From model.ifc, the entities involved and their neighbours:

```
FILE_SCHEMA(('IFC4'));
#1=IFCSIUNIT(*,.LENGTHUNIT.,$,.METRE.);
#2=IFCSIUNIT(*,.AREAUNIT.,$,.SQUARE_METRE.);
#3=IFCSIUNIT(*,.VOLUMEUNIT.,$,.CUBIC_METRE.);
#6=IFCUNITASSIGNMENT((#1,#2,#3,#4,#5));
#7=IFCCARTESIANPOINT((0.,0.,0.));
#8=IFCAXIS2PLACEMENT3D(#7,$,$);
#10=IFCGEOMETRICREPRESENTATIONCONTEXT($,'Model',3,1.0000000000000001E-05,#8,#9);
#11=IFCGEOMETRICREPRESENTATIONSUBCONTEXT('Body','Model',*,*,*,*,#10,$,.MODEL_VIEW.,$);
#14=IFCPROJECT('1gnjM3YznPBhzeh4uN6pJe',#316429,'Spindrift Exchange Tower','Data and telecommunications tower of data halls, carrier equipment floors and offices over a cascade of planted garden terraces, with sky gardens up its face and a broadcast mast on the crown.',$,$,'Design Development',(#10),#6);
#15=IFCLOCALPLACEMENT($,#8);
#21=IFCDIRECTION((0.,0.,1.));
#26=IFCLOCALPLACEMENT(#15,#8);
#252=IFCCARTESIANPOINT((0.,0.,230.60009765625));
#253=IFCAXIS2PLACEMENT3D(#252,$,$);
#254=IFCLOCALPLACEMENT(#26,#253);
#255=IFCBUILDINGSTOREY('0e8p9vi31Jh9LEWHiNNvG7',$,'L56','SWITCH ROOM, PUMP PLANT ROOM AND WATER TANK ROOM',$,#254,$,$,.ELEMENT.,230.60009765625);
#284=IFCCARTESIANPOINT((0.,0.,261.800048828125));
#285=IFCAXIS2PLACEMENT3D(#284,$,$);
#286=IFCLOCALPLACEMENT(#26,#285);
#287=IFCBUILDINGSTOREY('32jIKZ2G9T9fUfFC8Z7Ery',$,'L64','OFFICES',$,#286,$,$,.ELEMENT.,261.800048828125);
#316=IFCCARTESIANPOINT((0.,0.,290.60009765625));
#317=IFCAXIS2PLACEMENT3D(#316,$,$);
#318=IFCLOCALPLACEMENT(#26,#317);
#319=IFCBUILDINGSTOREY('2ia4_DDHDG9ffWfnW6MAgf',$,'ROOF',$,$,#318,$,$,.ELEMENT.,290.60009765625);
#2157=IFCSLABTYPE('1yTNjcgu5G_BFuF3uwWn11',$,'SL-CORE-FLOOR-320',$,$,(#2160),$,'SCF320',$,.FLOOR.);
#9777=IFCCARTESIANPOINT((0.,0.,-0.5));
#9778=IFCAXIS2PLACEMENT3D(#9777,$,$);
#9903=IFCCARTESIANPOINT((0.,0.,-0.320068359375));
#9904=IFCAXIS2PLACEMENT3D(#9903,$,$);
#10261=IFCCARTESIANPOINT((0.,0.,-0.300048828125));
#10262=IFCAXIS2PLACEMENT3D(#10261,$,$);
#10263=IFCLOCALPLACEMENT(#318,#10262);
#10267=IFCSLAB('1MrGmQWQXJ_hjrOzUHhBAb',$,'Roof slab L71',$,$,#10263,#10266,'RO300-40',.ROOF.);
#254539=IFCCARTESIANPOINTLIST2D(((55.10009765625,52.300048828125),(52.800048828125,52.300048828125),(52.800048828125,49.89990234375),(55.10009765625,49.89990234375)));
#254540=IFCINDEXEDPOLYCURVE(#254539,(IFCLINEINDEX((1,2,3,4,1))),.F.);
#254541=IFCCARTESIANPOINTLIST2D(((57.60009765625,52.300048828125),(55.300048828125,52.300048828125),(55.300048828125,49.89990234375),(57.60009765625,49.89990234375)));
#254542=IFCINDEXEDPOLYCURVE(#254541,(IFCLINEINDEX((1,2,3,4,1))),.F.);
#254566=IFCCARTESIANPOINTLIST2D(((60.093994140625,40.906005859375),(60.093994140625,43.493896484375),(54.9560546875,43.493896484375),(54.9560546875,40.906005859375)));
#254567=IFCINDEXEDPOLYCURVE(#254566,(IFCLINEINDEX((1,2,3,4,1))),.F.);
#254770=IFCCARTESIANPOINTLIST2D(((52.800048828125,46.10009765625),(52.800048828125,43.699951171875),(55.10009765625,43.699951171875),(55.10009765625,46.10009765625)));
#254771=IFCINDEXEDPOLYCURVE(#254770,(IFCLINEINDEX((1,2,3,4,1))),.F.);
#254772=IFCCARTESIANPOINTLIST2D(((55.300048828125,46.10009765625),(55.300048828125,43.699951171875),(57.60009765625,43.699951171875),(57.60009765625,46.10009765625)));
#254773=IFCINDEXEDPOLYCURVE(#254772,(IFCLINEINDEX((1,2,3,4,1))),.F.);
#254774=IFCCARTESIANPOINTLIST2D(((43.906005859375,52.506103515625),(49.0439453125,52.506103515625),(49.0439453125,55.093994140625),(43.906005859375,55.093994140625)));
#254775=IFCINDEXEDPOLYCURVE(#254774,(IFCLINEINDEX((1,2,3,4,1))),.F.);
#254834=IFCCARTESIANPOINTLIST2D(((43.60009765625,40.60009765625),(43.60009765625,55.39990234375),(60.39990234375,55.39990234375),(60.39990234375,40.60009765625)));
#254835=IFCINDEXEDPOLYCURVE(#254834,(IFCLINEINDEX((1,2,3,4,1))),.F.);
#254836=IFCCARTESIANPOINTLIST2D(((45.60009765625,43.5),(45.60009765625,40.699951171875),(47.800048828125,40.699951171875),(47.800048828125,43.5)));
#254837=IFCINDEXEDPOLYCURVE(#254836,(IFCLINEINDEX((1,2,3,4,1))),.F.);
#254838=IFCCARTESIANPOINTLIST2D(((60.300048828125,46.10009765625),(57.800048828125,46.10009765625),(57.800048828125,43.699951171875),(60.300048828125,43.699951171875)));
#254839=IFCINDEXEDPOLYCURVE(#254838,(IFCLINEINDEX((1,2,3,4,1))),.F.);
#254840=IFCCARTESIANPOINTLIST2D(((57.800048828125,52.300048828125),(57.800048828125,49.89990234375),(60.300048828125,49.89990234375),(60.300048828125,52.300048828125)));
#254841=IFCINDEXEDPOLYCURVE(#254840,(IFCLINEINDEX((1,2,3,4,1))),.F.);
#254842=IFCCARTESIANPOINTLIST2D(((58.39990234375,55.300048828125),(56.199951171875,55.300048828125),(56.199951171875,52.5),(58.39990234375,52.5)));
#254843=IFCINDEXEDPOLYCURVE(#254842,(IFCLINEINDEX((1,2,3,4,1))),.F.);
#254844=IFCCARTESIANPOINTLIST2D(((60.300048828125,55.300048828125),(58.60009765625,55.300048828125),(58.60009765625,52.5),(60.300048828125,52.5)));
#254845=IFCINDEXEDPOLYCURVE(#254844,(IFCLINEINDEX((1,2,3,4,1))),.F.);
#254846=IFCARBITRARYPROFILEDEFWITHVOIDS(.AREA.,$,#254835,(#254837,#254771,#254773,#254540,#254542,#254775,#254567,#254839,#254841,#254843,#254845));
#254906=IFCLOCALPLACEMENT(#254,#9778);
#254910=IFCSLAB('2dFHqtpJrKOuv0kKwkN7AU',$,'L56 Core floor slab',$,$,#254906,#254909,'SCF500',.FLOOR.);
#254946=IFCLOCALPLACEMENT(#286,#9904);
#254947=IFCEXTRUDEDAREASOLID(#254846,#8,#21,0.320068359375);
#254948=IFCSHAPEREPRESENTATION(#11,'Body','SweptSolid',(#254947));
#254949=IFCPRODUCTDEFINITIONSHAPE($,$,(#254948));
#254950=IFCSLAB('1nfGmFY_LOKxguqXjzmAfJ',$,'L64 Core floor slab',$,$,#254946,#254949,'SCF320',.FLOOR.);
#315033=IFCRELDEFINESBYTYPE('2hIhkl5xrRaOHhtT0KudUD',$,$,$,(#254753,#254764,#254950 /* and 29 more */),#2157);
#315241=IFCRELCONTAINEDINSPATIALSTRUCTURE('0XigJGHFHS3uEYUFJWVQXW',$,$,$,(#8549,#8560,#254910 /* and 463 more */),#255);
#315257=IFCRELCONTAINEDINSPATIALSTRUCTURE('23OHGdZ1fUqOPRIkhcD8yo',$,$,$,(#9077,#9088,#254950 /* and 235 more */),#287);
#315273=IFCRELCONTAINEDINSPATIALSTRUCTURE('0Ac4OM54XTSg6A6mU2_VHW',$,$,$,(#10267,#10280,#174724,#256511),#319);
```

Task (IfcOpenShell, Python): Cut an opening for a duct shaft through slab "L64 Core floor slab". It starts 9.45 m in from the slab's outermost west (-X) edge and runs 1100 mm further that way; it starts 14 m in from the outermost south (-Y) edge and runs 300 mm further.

```python
import numpy as np
import ifcopenshell
import ifcopenshell.api.feature
import ifcopenshell.api.geometry
import ifcopenshell.api.root
import ifcopenshell.geom
import ifcopenshell.util.placement
import ifcopenshell.util.representation
import ifcopenshell.util.shape
import ifcopenshell.util.unit

model = ifcopenshell.open("model.ifc")
unit_scale = ifcopenshell.util.unit.calculate_unit_scale(model)
settings = ifcopenshell.geom.settings()


def volume(element):
    """Net volume in cubic metres, openings subtracted."""
    shape = ifcopenshell.geom.create_shape(settings, element)
    return ifcopenshell.util.shape.get_volume(shape.geometry)


slab = model.by_id(254950)
before = volume(slab)

# Extent in the slab's own axes, in metres. The edges named are its -X and -Y sides.
slab_shape = ifcopenshell.geom.create_shape(settings, slab)
vertices = ifcopenshell.util.shape.get_vertices(slab_shape.geometry)
x_min, y_min, bottom = vertices.min(axis=0)
top = vertices[:, 2].max()

opening = ifcopenshell.api.root.create_entity(model, ifc_class="IfcOpeningElement", name="Duct shaft opening", predefined_type="OPENING")
context = ifcopenshell.util.representation.get_context(model, "Model", "Body", "MODEL_VIEW")
width, depth = 1.1, 0.3
outline = [(0.0, 0.0), (width, 0.0), (width, depth), (0.0, depth), (0.0, 0.0)]
# Overshoot both faces by 50 mm so the cut is clean.
shape = ifcopenshell.api.geometry.add_slab_representation(
    model, context=context, depth=top - bottom + 0.1, polyline=outline
)
ifcopenshell.api.geometry.assign_representation(model, product=opening, representation=shape)

matrix = ifcopenshell.util.placement.get_local_placement(slab.ObjectPlacement)
matrix[:, 3] = matrix @ np.append(np.array([x_min + 9.45, y_min + 14, bottom - 0.05]) / unit_scale, 1.0)
ifcopenshell.api.geometry.edit_object_placement(model, product=opening, matrix=matrix, is_si=False)
ifcopenshell.api.feature.add_feature(model, feature=opening, element=slab)

after = volume(slab)

print(f"slab volume {before:.3f} -> {after:.3f} m3")

model.write("model_rev.ifc")
```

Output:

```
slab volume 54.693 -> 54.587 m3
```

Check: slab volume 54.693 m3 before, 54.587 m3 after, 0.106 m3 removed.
